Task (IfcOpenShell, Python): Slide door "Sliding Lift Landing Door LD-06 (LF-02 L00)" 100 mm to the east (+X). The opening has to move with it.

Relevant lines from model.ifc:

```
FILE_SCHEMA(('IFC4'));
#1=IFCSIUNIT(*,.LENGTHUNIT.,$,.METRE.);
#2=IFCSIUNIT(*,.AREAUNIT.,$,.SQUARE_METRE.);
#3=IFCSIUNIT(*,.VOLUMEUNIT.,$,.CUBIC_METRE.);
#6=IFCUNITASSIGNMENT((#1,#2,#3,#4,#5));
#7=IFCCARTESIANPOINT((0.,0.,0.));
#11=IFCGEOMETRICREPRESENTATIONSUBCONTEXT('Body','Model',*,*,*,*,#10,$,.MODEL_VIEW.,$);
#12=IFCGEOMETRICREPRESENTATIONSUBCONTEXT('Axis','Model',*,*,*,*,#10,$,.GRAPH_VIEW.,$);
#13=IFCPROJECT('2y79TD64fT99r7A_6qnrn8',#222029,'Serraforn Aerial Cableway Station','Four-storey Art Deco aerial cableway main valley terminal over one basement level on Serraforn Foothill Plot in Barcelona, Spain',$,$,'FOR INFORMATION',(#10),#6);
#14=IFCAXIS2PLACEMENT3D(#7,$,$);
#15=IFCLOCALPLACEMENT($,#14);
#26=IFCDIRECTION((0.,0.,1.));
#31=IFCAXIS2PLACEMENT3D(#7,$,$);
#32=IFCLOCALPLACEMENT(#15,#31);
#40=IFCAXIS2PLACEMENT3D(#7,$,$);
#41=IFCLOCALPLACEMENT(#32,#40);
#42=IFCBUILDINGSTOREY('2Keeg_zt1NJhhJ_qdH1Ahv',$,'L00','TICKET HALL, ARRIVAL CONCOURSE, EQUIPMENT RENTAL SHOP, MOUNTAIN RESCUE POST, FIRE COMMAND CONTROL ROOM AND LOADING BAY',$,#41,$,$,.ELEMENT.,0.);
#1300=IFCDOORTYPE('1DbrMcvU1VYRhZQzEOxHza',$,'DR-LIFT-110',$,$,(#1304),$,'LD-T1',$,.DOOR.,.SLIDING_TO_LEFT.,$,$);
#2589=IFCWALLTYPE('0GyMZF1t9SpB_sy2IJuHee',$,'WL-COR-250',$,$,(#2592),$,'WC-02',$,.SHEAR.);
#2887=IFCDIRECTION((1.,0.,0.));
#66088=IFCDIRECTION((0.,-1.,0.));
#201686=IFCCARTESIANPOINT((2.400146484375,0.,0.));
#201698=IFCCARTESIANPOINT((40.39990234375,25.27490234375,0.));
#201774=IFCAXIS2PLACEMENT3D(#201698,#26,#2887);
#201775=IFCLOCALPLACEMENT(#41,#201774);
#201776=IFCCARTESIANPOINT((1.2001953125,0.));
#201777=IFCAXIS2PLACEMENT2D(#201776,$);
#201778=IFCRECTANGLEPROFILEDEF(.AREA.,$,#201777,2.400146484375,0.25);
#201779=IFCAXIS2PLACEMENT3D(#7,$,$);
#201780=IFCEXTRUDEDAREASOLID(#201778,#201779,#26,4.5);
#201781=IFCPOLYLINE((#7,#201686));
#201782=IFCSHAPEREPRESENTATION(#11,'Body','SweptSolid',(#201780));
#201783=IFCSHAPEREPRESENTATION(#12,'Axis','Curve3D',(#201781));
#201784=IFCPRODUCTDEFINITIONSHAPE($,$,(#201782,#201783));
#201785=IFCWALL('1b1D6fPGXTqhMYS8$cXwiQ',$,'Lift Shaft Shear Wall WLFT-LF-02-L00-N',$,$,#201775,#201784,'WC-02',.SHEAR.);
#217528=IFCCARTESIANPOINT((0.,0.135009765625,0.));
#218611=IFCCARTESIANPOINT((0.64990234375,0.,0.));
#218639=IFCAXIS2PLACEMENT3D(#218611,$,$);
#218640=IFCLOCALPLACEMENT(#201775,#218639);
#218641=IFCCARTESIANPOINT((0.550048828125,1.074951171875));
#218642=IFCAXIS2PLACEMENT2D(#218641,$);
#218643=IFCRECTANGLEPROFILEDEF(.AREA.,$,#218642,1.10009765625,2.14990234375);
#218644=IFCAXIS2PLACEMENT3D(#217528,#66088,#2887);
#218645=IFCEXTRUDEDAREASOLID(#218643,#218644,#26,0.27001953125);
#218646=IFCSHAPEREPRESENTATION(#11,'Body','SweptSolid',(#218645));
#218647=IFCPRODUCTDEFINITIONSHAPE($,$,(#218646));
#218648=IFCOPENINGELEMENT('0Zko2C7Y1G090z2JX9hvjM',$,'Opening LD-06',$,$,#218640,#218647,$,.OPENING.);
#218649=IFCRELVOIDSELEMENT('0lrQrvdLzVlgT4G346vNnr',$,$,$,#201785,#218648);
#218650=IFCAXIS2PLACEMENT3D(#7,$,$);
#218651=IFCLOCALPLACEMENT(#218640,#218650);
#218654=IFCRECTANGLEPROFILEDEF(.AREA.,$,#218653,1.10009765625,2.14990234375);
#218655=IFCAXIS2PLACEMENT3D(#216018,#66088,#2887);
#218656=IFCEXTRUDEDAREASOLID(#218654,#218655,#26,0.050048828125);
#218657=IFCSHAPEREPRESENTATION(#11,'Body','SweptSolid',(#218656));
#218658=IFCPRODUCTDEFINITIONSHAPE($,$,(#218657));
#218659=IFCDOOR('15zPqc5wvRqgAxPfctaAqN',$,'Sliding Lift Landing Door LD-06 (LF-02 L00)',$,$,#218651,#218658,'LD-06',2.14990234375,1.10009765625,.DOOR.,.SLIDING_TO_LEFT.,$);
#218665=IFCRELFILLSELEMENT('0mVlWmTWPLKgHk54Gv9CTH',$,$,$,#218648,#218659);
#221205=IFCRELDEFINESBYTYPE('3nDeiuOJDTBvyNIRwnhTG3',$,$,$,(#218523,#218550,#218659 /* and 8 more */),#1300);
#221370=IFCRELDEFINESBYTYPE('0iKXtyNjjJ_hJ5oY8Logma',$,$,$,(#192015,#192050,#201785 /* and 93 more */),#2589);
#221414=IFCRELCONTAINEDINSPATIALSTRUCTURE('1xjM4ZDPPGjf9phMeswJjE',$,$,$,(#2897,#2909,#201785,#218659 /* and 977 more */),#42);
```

```python
import ifcopenshell
import ifcopenshell.api.geometry
import ifcopenshell.util.placement

model = ifcopenshell.open("model.ifc")

door = model.by_guid("15zPqc5wvRqgAxPfctaAqN")
opening = door.FillsVoids[0].RelatingOpeningElement
wall = opening.VoidsElements[0].RelatingBuildingElement

wall_matrix = ifcopenshell.util.placement.get_local_placement(wall.ObjectPlacement)
shift = wall_matrix[:3, 0] * 0.1
before = ifcopenshell.util.placement.get_local_placement(door.ObjectPlacement)[:3, 3].copy()

# The door is placed relative to its opening, so it follows when the opening moves.
matrix = ifcopenshell.util.placement.get_local_placement(opening.ObjectPlacement)
matrix[:3, 3] += shift
ifcopenshell.api.geometry.edit_object_placement(
    model, product=opening, matrix=matrix, is_si=False, should_transform_children=True
)

after = ifcopenshell.util.placement.get_local_placement(door.ObjectPlacement)[:3, 3]
print("door moved by", (after - before).round(3) + 0.0)

model.write("model-out.ifc")
```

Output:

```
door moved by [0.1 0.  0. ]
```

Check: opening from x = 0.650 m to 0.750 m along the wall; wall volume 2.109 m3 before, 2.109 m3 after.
